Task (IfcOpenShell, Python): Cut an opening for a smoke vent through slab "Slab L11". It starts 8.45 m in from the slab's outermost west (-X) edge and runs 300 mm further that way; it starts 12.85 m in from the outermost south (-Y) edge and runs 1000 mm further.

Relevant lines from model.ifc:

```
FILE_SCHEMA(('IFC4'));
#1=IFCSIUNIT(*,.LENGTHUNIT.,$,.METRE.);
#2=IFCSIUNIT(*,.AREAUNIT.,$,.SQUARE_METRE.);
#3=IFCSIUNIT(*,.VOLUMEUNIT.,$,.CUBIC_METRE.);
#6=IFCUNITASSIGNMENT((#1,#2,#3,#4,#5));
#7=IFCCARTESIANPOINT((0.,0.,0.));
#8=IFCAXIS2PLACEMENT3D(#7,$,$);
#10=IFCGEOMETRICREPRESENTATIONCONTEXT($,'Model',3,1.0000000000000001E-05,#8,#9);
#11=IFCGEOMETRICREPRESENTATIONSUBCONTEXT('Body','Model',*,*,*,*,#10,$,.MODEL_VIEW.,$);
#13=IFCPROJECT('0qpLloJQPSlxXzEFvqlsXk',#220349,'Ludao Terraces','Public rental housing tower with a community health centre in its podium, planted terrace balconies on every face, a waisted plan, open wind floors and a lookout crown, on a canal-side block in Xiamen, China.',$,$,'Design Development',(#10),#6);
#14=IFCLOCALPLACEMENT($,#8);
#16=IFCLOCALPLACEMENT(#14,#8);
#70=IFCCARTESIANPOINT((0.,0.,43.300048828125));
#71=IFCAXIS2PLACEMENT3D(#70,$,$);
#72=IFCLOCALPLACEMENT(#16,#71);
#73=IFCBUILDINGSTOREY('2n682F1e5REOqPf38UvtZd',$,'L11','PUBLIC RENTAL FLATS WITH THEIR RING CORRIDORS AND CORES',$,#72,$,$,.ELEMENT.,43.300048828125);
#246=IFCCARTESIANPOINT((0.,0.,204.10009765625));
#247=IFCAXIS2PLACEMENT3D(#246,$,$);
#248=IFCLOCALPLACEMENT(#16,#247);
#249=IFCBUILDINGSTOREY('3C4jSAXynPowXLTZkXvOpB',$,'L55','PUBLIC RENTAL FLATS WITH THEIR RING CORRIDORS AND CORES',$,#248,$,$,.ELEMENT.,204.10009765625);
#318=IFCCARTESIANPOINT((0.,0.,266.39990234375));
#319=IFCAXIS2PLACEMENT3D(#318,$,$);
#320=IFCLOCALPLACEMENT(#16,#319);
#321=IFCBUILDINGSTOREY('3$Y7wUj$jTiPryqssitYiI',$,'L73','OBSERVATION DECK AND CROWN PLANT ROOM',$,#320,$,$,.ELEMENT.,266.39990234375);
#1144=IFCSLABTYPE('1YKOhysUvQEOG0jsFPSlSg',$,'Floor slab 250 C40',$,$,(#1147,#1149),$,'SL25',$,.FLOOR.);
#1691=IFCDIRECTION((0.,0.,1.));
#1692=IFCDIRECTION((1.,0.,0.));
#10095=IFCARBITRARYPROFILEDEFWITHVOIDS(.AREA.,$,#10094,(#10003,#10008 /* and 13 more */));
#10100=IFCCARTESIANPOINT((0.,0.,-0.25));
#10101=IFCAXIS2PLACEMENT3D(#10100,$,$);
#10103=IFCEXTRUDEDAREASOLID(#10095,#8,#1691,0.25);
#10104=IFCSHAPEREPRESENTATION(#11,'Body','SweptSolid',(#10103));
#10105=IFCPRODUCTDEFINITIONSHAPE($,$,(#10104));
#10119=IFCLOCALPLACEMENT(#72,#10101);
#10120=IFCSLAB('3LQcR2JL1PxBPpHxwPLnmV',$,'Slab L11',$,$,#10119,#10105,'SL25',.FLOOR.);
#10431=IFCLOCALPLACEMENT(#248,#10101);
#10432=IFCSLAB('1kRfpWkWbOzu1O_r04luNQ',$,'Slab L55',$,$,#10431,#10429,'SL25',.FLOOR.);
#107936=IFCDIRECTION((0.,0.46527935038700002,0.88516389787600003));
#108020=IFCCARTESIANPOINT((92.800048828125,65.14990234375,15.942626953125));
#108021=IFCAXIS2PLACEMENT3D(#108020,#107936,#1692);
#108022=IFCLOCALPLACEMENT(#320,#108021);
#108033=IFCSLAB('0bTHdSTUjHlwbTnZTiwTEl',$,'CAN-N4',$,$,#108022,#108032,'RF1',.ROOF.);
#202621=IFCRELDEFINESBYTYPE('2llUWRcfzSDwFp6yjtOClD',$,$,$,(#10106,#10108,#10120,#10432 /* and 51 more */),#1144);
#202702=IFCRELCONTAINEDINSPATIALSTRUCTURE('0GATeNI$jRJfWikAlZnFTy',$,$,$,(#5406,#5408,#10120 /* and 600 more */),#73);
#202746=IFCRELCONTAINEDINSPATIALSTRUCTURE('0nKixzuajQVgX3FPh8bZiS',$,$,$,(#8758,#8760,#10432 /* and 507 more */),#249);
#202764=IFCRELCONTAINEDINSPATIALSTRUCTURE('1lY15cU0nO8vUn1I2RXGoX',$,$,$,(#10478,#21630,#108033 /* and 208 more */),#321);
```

```python
import numpy as np
import ifcopenshell
import ifcopenshell.api.feature
import ifcopenshell.api.geometry
import ifcopenshell.api.root
import ifcopenshell.geom
import ifcopenshell.util.placement
import ifcopenshell.util.representation
import ifcopenshell.util.shape
import ifcopenshell.util.unit

model = ifcopenshell.open("model.ifc")
unit_scale = ifcopenshell.util.unit.calculate_unit_scale(model)
settings = ifcopenshell.geom.settings()


def volume(element):
    """Net volume in cubic metres, openings subtracted."""
    shape = ifcopenshell.geom.create_shape(settings, element)
    return ifcopenshell.util.shape.get_volume(shape.geometry)


slab = model.by_guid("3LQcR2JL1PxBPpHxwPLnmV")
before = volume(slab)

# Extent in the slab's own axes, in metres. The edges named are its -X and -Y sides.
slab_shape = ifcopenshell.geom.create_shape(settings, slab)
vertices = ifcopenshell.util.shape.get_vertices(slab_shape.geometry)
x_min, y_min, bottom = vertices.min(axis=0)
top = vertices[:, 2].max()

opening = ifcopenshell.api.root.create_entity(model, ifc_class="IfcOpeningElement", name="Smoke vent opening", predefined_type="OPENING")
context = ifcopenshell.util.representation.get_context(model, "Model", "Body", "MODEL_VIEW")
width, depth = 0.3, 1
outline = [(0.0, 0.0), (width, 0.0), (width, depth), (0.0, depth), (0.0, 0.0)]
# Overshoot both faces by 50 mm so the cut is clean.
shape = ifcopenshell.api.geometry.add_slab_representation(
    model, context=context, depth=top - bottom + 0.1, polyline=outline
)
ifcopenshell.api.geometry.assign_representation(model, product=opening, representation=shape)

matrix = ifcopenshell.util.placement.get_local_placement(slab.ObjectPlacement)
matrix[:, 3] = matrix @ np.append(np.array([x_min + 8.45, y_min + 12.85, bottom - 0.05]) / unit_scale, 1.0)
ifcopenshell.api.geometry.edit_object_placement(model, product=opening, matrix=matrix, is_si=False)
ifcopenshell.api.feature.add_feature(model, feature=opening, element=slab)

after = volume(slab)

print(f"slab volume {before:.3f} -> {after:.3f} m3")

model.write("model_rev.ifc")
```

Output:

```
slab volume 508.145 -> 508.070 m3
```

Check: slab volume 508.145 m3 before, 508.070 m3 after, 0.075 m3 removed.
